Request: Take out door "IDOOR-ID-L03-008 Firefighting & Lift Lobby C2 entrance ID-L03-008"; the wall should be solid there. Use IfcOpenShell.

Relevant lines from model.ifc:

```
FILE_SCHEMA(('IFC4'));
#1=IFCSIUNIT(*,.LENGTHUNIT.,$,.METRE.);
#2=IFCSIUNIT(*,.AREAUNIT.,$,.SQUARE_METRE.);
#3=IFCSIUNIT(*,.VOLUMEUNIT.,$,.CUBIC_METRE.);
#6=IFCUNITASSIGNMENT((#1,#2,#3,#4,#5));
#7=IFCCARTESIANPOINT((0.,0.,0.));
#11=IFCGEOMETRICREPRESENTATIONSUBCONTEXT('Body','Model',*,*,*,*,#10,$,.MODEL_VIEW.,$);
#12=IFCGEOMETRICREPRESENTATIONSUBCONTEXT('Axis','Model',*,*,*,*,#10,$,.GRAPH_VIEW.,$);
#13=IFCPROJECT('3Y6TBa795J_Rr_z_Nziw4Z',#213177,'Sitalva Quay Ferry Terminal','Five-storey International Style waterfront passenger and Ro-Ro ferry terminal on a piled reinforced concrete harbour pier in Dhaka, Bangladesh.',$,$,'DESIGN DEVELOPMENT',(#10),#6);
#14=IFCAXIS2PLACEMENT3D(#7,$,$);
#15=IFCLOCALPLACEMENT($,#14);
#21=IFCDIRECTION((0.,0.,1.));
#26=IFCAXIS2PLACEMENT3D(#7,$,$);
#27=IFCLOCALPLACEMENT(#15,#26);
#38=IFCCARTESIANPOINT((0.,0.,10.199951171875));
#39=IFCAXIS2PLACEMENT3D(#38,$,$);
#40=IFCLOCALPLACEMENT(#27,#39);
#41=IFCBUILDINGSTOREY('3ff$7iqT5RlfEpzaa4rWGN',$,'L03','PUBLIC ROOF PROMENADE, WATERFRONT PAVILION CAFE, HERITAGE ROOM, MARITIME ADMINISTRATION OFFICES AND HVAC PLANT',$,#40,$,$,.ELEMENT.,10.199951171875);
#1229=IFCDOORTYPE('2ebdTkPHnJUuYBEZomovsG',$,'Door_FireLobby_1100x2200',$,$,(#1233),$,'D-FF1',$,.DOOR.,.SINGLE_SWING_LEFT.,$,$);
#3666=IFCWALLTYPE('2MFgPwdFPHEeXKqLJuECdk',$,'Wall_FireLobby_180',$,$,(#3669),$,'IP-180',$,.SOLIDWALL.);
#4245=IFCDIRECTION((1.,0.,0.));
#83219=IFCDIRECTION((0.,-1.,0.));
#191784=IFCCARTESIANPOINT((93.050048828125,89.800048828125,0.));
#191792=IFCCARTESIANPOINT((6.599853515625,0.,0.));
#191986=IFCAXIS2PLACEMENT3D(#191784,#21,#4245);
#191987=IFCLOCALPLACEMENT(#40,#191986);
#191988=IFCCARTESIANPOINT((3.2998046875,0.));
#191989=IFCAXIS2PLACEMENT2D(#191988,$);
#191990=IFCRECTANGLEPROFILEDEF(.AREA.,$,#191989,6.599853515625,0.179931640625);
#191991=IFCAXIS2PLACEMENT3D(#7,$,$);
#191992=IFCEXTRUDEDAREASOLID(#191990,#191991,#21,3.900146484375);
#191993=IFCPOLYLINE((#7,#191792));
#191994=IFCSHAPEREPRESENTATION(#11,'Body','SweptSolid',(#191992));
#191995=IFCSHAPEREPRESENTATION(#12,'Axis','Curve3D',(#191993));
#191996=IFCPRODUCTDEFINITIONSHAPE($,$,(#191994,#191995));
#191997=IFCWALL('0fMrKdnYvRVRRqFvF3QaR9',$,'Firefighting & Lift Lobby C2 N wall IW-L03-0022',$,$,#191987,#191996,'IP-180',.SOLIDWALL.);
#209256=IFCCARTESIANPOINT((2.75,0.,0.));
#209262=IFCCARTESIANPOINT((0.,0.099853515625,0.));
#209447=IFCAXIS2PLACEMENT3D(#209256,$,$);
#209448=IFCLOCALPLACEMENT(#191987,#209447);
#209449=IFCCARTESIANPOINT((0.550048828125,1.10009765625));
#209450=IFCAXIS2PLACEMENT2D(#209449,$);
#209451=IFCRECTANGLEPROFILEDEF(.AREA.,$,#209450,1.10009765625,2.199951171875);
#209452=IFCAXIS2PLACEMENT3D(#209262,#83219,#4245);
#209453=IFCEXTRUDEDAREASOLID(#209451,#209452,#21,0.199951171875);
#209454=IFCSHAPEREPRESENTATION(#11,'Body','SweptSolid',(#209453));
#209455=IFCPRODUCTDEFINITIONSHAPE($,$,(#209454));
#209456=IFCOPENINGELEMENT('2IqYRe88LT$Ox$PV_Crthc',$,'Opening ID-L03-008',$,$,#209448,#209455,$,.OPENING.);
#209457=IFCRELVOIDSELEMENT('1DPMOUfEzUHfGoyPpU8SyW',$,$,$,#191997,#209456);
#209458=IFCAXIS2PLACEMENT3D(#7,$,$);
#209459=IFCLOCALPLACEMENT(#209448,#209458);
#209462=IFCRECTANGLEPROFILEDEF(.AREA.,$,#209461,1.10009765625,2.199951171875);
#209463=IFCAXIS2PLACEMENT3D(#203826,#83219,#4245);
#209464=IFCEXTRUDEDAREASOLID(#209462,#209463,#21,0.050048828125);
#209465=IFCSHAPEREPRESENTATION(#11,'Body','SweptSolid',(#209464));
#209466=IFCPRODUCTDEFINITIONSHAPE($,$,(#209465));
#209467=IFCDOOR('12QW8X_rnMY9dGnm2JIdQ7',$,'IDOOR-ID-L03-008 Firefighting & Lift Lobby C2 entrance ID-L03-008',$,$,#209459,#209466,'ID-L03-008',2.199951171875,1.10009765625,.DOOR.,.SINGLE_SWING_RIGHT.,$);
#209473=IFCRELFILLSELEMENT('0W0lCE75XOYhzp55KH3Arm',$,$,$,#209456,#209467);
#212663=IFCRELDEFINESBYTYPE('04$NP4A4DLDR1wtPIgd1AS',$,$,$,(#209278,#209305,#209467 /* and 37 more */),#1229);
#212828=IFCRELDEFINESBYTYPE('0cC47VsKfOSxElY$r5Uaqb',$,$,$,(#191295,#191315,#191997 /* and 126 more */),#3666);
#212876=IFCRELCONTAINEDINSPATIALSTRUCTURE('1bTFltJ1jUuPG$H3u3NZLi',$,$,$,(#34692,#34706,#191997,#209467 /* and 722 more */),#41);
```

```python
import ifcopenshell
import ifcopenshell.api.feature
import ifcopenshell.api.root
import ifcopenshell.geom
import ifcopenshell.util.shape

model = ifcopenshell.open("model.ifc")
settings = ifcopenshell.geom.settings()


def volume(element):
    """Net volume in cubic metres, openings subtracted."""
    shape = ifcopenshell.geom.create_shape(settings, element)
    return ifcopenshell.util.shape.get_volume(shape.geometry)


door = model.by_id(209467)
opening = door.FillsVoids[0].RelatingOpeningElement
wall = opening.VoidsElements[0].RelatingBuildingElement
before = volume(wall)

ifcopenshell.api.root.remove_product(model, product=door)
ifcopenshell.api.feature.remove_feature(model, feature=opening)

after = volume(wall)

print(f"wall volume {before:.3f} -> {after:.3f} m3")

model.write("model_edited.ifc")
```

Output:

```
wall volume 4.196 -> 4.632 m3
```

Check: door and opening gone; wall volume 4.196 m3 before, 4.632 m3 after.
